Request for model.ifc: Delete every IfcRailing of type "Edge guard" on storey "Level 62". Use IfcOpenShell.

First a look at what the model holds.

```python
import ifcopenshell
import ifcopenshell.util.element

model = ifcopenshell.open("model.ifc")
print(model.schema)
storey = next(s for s in model.by_type("IfcBuildingStorey") if s.Name == "Level 62")
railings = [e for e in ifcopenshell.util.element.get_decomposition(storey) if e.is_a("IfcRailing")]
seen = {}
for e in railings:
    element_type = ifcopenshell.util.element.get_type(e)
    name = element_type.Name if element_type not in (None, e) else None
    seen[name] = seen.get(name, 0) + 1
for name, count in sorted(seen.items(), key=str):
    print(count, "x", name)
```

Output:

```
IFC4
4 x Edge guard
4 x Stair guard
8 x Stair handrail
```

```python
import ifcopenshell
import ifcopenshell.api.root
import ifcopenshell.util.element

model = ifcopenshell.open("model.ifc")

storey = next(s for s in model.by_type("IfcBuildingStorey") if s.Name == "Level 62")
railings = [e for e in ifcopenshell.util.element.get_decomposition(storey) if e.is_a("IfcRailing")]
targets = [e for e in railings if (t := ifcopenshell.util.element.get_type(e)) not in (None, e) and t.Name == "Edge guard"]

for e in targets:
    ifcopenshell.api.root.remove_product(model, product=e)
print(len(targets), "removed")

model.write("model_rev.ifc")
```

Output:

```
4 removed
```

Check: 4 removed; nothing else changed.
